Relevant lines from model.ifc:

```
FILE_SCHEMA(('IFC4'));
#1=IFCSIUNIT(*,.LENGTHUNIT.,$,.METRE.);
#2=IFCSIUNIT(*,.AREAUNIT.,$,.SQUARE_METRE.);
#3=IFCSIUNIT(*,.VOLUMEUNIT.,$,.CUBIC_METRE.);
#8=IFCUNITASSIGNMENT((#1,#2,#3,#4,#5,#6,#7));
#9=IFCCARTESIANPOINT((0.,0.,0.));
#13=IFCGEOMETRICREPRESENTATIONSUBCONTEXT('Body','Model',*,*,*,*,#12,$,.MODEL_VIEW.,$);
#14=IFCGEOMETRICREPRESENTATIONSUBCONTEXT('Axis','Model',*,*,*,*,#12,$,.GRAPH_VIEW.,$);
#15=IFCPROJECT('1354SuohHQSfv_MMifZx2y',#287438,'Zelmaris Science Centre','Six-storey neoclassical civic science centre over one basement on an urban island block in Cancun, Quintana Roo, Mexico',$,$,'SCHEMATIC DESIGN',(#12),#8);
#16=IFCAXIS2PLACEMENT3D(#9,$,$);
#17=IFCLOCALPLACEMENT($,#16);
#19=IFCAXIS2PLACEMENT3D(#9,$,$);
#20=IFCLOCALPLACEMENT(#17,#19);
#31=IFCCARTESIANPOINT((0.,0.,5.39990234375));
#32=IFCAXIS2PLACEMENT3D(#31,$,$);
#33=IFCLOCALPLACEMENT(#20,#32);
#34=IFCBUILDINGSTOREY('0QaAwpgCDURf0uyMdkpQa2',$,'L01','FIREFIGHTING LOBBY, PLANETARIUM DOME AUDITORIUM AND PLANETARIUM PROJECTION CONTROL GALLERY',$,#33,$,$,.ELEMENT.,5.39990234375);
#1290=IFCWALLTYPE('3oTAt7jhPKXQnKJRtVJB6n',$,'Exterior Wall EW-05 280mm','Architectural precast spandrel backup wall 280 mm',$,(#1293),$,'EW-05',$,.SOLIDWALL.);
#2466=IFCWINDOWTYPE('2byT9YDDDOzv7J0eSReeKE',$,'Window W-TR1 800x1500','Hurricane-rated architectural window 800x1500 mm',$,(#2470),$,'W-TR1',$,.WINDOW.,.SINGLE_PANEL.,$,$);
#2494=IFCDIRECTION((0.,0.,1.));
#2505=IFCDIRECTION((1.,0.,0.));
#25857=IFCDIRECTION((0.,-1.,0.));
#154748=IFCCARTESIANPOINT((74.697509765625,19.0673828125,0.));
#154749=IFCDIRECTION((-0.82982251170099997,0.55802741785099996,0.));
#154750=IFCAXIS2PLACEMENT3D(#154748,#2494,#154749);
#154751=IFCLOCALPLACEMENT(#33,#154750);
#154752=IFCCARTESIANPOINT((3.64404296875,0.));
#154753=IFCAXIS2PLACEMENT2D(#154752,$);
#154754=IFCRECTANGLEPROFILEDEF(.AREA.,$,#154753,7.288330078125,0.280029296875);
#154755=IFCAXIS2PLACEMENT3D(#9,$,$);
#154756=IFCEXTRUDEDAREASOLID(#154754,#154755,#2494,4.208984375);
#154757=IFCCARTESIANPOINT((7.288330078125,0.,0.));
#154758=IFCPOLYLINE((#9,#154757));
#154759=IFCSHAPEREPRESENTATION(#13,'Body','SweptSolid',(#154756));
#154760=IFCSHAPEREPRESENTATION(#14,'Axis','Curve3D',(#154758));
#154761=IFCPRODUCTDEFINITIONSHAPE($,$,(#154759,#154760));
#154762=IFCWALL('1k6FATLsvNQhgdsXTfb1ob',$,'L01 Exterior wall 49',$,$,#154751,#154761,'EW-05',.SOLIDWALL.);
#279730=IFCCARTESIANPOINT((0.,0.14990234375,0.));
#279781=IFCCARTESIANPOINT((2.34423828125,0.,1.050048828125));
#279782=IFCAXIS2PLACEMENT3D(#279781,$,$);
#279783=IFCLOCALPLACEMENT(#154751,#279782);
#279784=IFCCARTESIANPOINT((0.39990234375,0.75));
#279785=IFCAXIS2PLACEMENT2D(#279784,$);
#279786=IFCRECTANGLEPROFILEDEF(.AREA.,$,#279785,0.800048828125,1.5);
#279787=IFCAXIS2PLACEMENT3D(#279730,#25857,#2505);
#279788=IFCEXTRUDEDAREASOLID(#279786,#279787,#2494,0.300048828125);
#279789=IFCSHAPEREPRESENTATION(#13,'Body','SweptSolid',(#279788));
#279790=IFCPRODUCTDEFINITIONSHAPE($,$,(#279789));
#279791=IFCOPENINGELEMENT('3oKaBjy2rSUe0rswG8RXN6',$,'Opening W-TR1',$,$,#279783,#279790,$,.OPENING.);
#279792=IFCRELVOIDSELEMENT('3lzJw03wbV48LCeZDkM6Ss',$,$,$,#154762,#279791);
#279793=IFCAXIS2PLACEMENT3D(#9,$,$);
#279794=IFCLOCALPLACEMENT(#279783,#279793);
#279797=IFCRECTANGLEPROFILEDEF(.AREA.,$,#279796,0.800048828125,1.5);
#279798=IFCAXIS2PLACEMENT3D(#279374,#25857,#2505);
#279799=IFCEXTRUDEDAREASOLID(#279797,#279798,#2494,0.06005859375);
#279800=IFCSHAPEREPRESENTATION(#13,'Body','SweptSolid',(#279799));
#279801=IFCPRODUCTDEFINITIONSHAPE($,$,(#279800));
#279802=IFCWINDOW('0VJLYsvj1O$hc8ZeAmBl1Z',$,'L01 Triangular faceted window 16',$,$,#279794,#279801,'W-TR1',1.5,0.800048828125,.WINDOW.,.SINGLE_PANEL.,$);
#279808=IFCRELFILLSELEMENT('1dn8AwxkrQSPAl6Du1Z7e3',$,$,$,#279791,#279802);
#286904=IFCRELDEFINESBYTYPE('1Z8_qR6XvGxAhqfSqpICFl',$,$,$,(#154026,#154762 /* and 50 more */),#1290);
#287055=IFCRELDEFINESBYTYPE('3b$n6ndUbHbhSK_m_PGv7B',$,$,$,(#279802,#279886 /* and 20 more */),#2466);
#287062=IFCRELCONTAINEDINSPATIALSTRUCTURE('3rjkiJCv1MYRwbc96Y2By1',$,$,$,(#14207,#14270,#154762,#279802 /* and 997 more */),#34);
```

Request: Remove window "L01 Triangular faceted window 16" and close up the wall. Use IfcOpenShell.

```python
import ifcopenshell
import ifcopenshell.api.feature
import ifcopenshell.api.root
import ifcopenshell.geom
import ifcopenshell.util.shape

model = ifcopenshell.open("model.ifc")
settings = ifcopenshell.geom.settings()


def volume(element):
    """Net volume in cubic metres, openings subtracted."""
    shape = ifcopenshell.geom.create_shape(settings, element)
    return ifcopenshell.util.shape.get_volume(shape.geometry)


window = model.by_guid("0VJLYsvj1O$hc8ZeAmBl1Z")
opening = window.FillsVoids[0].RelatingOpeningElement
wall = opening.VoidsElements[0].RelatingBuildingElement
before = volume(wall)

ifcopenshell.api.root.remove_product(model, product=window)
ifcopenshell.api.feature.remove_feature(model, feature=opening)

after = volume(wall)

print(f"wall volume {before:.3f} -> {after:.3f} m3")

model.write("model_updated.ifc")
```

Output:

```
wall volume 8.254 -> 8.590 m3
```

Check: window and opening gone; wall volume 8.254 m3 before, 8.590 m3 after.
